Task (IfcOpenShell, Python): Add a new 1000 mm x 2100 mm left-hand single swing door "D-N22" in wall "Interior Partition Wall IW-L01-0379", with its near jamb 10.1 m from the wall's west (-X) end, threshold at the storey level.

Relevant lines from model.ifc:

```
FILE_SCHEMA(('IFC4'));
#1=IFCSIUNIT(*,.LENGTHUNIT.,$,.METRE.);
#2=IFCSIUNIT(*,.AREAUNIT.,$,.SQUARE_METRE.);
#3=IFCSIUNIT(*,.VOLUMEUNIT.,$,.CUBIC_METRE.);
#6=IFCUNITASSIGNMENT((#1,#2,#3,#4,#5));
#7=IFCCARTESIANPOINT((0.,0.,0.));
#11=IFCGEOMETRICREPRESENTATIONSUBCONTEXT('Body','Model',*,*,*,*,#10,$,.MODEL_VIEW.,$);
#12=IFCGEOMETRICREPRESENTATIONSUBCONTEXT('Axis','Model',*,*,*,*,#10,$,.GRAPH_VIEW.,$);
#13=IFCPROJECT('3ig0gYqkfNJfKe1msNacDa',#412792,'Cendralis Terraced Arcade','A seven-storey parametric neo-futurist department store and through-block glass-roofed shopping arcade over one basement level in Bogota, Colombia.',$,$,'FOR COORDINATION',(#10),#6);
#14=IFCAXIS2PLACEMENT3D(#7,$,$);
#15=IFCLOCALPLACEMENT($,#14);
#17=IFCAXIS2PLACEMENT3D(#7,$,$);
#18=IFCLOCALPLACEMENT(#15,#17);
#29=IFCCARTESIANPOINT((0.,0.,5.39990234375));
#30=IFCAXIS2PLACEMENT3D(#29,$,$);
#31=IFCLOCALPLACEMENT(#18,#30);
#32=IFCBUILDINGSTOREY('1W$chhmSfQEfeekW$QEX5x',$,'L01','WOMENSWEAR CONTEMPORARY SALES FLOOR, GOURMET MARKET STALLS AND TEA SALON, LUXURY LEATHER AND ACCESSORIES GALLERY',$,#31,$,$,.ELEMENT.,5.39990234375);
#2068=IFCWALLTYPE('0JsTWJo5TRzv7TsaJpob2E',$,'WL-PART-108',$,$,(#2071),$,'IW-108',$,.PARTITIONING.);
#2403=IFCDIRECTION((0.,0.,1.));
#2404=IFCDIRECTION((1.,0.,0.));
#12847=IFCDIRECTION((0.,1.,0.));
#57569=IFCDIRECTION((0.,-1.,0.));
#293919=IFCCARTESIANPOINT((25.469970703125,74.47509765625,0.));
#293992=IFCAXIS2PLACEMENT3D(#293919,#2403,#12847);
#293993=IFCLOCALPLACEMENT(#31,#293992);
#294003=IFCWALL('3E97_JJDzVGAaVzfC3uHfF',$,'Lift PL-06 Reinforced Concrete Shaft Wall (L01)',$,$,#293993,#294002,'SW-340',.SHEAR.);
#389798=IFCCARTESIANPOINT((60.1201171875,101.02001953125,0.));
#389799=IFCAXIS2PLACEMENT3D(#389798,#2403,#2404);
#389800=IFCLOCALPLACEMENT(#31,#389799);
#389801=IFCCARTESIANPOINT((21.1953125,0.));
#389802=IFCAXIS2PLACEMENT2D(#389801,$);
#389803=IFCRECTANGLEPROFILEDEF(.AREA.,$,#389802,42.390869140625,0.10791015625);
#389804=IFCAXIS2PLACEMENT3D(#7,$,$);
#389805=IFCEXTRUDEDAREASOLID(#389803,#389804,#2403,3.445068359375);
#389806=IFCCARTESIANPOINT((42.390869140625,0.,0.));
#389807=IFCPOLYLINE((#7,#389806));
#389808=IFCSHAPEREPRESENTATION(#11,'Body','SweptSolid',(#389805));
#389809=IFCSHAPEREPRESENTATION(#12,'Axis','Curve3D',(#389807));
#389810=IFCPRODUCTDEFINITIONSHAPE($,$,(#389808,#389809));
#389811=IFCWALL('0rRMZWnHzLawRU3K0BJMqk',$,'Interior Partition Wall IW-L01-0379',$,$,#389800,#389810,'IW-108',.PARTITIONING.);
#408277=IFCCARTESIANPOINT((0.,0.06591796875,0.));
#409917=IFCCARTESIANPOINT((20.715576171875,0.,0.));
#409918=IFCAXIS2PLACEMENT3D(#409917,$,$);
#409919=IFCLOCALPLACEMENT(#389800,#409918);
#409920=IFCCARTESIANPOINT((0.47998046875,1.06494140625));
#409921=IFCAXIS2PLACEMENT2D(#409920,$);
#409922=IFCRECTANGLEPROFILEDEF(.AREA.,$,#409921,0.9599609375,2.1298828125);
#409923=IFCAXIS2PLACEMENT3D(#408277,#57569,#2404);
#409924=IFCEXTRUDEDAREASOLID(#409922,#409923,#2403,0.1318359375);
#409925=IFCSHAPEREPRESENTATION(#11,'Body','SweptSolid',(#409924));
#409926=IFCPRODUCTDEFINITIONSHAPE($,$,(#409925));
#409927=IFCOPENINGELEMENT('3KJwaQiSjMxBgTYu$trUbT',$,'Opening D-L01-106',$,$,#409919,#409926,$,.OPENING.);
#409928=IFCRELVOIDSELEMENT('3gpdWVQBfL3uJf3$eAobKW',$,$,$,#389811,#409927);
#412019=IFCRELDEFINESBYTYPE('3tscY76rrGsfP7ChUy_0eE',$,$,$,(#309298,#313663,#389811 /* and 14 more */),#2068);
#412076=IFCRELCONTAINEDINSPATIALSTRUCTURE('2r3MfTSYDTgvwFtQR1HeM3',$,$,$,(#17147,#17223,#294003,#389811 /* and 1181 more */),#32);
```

```python
import numpy as np
import ifcopenshell
import ifcopenshell.api.feature
import ifcopenshell.api.geometry
import ifcopenshell.api.root
import ifcopenshell.api.spatial
import ifcopenshell.geom
import ifcopenshell.util.element
import ifcopenshell.util.placement
import ifcopenshell.util.representation
import ifcopenshell.util.shape
import ifcopenshell.util.unit

model = ifcopenshell.open("model.ifc")
unit_scale = ifcopenshell.util.unit.calculate_unit_scale(model)
settings = ifcopenshell.geom.settings()


def volume(element):
    """Net volume in cubic metres, openings subtracted."""
    shape = ifcopenshell.geom.create_shape(settings, element)
    return ifcopenshell.util.shape.get_volume(shape.geometry)


wall = model.by_guid("0rRMZWnHzLawRU3K0BJMqk")
storey = ifcopenshell.util.element.get_container(wall, ifc_class="IfcBuildingStorey")
context = ifcopenshell.util.representation.get_context(model, "Model", "Body", "MODEL_VIEW")
before = volume(wall)

width, height, from_end, sill = 1, 2.1, 10.1, 0.0  # metres

# The wall runs along its own X axis, and the end named is its -X end.
wall_shape = ifcopenshell.geom.create_shape(settings, wall)
x, y, z = ifcopenshell.util.shape.get_vertices(wall_shape.geometry).T
start = x.min() + from_end
face, thickness = float(y.min()), float(y.max() - y.min())
wall_matrix = ifcopenshell.util.placement.get_local_placement(wall.ObjectPlacement)
level = ifcopenshell.util.placement.get_local_placement(storey.ObjectPlacement)[2, 3]


def in_wall(x, y):
    """Placement at x, y metres in the wall's axes, at sill height."""
    matrix = wall_matrix.copy()
    matrix[:, 3] = wall_matrix @ np.array([x / unit_scale, y / unit_scale, 0.0, 1.0])
    matrix[2, 3] = level + sill / unit_scale
    return matrix


# Opening: a box that overshoots both wall faces by 50 mm.
opening = ifcopenshell.api.root.create_entity(model, ifc_class="IfcOpeningElement", predefined_type="OPENING")
box = ifcopenshell.api.geometry.add_wall_representation(
    model, context=context, length=width, height=height, thickness=thickness + 0.1
)
ifcopenshell.api.geometry.assign_representation(model, product=opening, representation=box)
ifcopenshell.api.geometry.edit_object_placement(model, product=opening, matrix=in_wall(start, face - 0.05), is_si=False)
ifcopenshell.api.feature.add_feature(model, feature=opening, element=wall)

door = ifcopenshell.api.root.create_entity(model, ifc_class="IfcDoor", name="D-N22", predefined_type="DOOR")
door.OverallWidth, door.OverallHeight = width / unit_scale, height / unit_scale
door.OperationType = "SINGLE_SWING_LEFT"
body = ifcopenshell.api.geometry.add_door_representation(
    model,
    context=context,
    overall_width=door.OverallWidth,
    overall_height=door.OverallHeight,
    operation_type="SINGLE_SWING_LEFT",
    lining_properties={"LiningDepth": thickness / unit_scale, "ThresholdDepth": thickness / unit_scale},
)
ifcopenshell.api.geometry.assign_representation(model, product=door, representation=body)
ifcopenshell.api.spatial.assign_container(model, products=[door], relating_structure=storey)
ifcopenshell.api.feature.add_filling(model, opening=opening, element=door)

# The lining spans the wall, so the door starts at the wall face.
ifcopenshell.api.geometry.edit_object_placement(model, product=door, matrix=in_wall(start, face), is_si=False)

after = volume(wall)

print(f"wall volume {before:.3f} -> {after:.3f} m3")

model.write("model_rev.ifc")
```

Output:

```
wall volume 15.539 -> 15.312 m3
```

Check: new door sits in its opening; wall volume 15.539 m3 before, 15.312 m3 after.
